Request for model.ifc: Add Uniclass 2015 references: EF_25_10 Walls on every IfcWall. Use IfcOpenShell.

First a look at what the model holds.

```python
import ifcopenshell

model = ifcopenshell.open("model.ifc")
print(model.schema)
print("classifications:", [c.Name for c in model.by_type("IfcClassification")])
for ifc_class in ("IfcDoor", "IfcRoof", "IfcStair", "IfcWall", "IfcWindow"):
    print(ifc_class, len(model.by_type(ifc_class)))
```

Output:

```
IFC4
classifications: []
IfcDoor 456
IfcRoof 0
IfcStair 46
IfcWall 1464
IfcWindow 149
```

```python
import ifcopenshell
import ifcopenshell.api.classification

model = ifcopenshell.open("model.ifc")

system = ifcopenshell.api.classification.add_classification(model, classification="Uniclass 2015")

codes = {
    "IfcWall": ("EF_25_10", "Walls"),
}
for ifc_class, (code, name) in codes.items():
    products = model.by_type(ifc_class)
    ifcopenshell.api.classification.add_reference(
        model, products=products, classification=system, identification=code, name=name
    )
    print(code, len(products))

model.write("model_rev.ifc")
```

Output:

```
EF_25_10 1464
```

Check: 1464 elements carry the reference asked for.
